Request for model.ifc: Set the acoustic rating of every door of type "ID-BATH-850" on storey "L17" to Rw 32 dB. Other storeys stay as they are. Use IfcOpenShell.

First a look at what the model holds.

```python
import ifcopenshell
import ifcopenshell.util.element

model = ifcopenshell.open("model.ifc")
print(model.schema)
storey = next(s for s in model.by_type("IfcBuildingStorey") if s.Name == "L17")
doors = [e for e in ifcopenshell.util.element.get_decomposition(storey) if e.is_a("IfcDoor")]
seen = {}
for e in doors:
    element_type = ifcopenshell.util.element.get_type(e)
    key = (element_type.Name if element_type != e and element_type else None, ifcopenshell.util.element.get_pset(e, "Pset_DoorCommon", "AcousticRating"))
    seen[key] = seen.get(key, 0) + 1
for (name, value), count in sorted(seen.items(), key=str):
    print(count, "x", name, "|", value)
```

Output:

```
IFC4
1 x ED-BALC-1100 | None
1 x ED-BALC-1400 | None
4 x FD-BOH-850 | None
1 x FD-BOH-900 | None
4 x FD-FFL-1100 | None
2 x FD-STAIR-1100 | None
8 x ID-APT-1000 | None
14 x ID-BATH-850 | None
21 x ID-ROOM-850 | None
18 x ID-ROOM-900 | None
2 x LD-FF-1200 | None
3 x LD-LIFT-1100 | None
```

```python
import ifcopenshell
import ifcopenshell.api.pset
import ifcopenshell.util.element

model = ifcopenshell.open("model.ifc")

storey = next(s for s in model.by_type("IfcBuildingStorey") if s.Name == "L17")
doors = [e for e in ifcopenshell.util.element.get_decomposition(storey) if e.is_a("IfcDoor")]

count = 0
for e in doors:
    element_type = ifcopenshell.util.element.get_type(e)
    if element_type in (None, e) or element_type.Name != "ID-BATH-850":
        continue
    found = ifcopenshell.util.element.get_pset(e, "Pset_DoorCommon", should_inherit=False)
    if found:
        pset = model.by_id(found["id"])
        if len(ifcopenshell.util.element.get_elements_by_pset(pset)) > 1:
            pset = ifcopenshell.api.pset.unshare_pset(model, products=[e], pset=pset)[0]
    else:
        pset = ifcopenshell.api.pset.add_pset(model, product=e, name="Pset_DoorCommon")
    ifcopenshell.api.pset.edit_pset(model, pset=pset, properties={"AcousticRating": "Rw 32 dB"})
    count += 1

print(count, "doors updated")

model.write("model_rev.ifc")
```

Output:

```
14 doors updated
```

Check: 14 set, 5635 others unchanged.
